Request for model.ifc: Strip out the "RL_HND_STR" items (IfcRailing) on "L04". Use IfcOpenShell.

First a look at what the model holds.

```python
import ifcopenshell
import ifcopenshell.util.element

model = ifcopenshell.open("model.ifc")
print(model.schema)
storey = next(s for s in model.by_type("IfcBuildingStorey") if s.Name == "L04")
railings = [e for e in ifcopenshell.util.element.get_decomposition(storey) if e.is_a("IfcRailing")]
seen = {}
for e in railings:
    element_type = ifcopenshell.util.element.get_type(e)
    name = element_type.Name if element_type not in (None, e) else None
    seen[name] = seen.get(name, 0) + 1
for name, count in sorted(seen.items(), key=str):
    print(count, "x", name)
```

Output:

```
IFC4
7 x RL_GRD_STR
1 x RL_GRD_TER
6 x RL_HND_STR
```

```python
import ifcopenshell
import ifcopenshell.api.root
import ifcopenshell.util.element

model = ifcopenshell.open("model.ifc")

storey = next(s for s in model.by_type("IfcBuildingStorey") if s.Name == "L04")
railings = [e for e in ifcopenshell.util.element.get_decomposition(storey) if e.is_a("IfcRailing")]
targets = [e for e in railings if (t := ifcopenshell.util.element.get_type(e)) not in (None, e) and t.Name == "RL_HND_STR"]

for e in targets:
    ifcopenshell.api.root.remove_product(model, product=e)
print(len(targets), "removed")

model.write("model_v2.ifc")
```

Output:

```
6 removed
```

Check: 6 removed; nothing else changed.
